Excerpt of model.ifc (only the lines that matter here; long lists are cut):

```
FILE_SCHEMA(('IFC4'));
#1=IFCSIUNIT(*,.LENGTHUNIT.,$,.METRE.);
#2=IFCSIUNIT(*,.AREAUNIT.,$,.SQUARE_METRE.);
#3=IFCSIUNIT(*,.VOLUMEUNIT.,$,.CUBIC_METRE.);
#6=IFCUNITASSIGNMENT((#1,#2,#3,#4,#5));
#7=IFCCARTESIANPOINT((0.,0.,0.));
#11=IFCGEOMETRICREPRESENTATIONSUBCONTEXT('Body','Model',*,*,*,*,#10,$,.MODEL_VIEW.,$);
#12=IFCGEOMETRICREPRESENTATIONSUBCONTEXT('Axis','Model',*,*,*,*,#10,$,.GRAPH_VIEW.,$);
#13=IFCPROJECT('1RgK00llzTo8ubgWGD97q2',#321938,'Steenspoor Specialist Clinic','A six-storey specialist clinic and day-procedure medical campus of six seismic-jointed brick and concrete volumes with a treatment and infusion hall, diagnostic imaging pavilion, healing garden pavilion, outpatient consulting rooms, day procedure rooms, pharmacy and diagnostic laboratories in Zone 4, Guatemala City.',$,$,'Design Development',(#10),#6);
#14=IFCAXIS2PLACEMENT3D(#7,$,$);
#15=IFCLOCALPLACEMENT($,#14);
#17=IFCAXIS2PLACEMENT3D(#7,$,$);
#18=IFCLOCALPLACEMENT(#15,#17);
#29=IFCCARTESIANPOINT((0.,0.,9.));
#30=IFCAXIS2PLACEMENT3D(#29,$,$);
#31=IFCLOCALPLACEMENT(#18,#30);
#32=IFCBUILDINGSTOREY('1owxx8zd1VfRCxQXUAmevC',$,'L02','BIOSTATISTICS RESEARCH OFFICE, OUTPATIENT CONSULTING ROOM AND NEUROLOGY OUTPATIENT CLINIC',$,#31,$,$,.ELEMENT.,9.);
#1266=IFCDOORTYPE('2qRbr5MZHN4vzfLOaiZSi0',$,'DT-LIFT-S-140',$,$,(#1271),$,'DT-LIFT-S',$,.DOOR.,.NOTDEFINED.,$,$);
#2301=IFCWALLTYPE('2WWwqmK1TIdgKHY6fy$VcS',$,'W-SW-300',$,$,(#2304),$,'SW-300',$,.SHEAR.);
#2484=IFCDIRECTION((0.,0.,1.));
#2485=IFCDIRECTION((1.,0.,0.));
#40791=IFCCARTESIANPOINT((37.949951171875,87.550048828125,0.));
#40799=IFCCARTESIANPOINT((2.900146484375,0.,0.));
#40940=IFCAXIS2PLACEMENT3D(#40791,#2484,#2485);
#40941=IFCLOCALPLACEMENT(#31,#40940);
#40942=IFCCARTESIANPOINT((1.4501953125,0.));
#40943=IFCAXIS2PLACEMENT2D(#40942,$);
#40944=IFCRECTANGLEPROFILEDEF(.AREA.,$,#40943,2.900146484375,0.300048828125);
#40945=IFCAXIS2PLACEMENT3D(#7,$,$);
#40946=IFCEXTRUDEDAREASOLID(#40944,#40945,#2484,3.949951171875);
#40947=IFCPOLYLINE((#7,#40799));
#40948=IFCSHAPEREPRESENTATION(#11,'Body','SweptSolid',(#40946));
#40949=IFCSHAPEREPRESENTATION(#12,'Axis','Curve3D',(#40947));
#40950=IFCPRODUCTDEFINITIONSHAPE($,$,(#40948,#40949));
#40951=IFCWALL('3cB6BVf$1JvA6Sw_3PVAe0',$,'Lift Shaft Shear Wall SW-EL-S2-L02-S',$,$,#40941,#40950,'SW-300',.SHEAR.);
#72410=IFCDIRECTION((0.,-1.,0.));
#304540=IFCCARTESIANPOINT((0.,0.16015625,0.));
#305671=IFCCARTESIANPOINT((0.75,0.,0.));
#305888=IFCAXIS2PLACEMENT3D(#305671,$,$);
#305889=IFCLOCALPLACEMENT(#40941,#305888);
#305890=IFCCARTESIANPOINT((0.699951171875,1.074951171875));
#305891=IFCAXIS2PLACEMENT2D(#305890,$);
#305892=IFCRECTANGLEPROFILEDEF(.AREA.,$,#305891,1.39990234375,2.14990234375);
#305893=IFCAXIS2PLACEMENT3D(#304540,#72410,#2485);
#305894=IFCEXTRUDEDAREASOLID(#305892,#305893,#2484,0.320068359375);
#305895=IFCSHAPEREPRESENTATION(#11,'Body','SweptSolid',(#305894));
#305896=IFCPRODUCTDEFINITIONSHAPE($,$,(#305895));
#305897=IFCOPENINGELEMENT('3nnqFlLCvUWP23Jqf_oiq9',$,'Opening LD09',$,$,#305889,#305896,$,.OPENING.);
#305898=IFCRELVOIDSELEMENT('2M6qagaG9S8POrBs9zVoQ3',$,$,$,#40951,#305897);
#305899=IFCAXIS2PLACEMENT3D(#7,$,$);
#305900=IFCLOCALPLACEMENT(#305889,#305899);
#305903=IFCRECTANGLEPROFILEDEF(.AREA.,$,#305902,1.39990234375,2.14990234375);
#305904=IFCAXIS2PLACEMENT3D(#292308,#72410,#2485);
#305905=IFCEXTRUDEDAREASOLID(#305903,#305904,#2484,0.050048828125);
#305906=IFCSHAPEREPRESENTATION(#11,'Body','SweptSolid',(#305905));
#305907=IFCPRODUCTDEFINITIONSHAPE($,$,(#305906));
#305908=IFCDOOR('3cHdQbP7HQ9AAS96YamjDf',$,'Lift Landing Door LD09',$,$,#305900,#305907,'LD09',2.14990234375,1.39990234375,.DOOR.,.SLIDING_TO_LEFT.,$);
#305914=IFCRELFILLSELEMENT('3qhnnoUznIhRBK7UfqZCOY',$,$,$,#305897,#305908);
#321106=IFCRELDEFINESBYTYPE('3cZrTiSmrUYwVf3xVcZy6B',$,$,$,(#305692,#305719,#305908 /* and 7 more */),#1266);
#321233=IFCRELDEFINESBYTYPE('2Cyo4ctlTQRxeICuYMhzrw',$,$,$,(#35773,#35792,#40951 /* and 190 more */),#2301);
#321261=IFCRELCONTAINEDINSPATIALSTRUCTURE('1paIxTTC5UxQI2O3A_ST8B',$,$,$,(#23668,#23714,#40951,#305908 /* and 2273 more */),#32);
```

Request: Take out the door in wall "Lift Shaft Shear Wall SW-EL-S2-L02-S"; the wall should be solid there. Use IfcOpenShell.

```python
import ifcopenshell
import ifcopenshell.api.feature
import ifcopenshell.api.root
import ifcopenshell.geom
import ifcopenshell.util.shape

model = ifcopenshell.open("model.ifc")
settings = ifcopenshell.geom.settings()


def volume(element):
    """Net volume in cubic metres, openings subtracted."""
    shape = ifcopenshell.geom.create_shape(settings, element)
    return ifcopenshell.util.shape.get_volume(shape.geometry)


door = model.by_id(305908)
opening = door.FillsVoids[0].RelatingOpeningElement
wall = opening.VoidsElements[0].RelatingBuildingElement
before = volume(wall)

ifcopenshell.api.root.remove_product(model, product=door)
ifcopenshell.api.feature.remove_feature(model, feature=opening)

after = volume(wall)

print(f"wall volume {before:.3f} -> {after:.3f} m3")

model.write("model_edited.ifc")
```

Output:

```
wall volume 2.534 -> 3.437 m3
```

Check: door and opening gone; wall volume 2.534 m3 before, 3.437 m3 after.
